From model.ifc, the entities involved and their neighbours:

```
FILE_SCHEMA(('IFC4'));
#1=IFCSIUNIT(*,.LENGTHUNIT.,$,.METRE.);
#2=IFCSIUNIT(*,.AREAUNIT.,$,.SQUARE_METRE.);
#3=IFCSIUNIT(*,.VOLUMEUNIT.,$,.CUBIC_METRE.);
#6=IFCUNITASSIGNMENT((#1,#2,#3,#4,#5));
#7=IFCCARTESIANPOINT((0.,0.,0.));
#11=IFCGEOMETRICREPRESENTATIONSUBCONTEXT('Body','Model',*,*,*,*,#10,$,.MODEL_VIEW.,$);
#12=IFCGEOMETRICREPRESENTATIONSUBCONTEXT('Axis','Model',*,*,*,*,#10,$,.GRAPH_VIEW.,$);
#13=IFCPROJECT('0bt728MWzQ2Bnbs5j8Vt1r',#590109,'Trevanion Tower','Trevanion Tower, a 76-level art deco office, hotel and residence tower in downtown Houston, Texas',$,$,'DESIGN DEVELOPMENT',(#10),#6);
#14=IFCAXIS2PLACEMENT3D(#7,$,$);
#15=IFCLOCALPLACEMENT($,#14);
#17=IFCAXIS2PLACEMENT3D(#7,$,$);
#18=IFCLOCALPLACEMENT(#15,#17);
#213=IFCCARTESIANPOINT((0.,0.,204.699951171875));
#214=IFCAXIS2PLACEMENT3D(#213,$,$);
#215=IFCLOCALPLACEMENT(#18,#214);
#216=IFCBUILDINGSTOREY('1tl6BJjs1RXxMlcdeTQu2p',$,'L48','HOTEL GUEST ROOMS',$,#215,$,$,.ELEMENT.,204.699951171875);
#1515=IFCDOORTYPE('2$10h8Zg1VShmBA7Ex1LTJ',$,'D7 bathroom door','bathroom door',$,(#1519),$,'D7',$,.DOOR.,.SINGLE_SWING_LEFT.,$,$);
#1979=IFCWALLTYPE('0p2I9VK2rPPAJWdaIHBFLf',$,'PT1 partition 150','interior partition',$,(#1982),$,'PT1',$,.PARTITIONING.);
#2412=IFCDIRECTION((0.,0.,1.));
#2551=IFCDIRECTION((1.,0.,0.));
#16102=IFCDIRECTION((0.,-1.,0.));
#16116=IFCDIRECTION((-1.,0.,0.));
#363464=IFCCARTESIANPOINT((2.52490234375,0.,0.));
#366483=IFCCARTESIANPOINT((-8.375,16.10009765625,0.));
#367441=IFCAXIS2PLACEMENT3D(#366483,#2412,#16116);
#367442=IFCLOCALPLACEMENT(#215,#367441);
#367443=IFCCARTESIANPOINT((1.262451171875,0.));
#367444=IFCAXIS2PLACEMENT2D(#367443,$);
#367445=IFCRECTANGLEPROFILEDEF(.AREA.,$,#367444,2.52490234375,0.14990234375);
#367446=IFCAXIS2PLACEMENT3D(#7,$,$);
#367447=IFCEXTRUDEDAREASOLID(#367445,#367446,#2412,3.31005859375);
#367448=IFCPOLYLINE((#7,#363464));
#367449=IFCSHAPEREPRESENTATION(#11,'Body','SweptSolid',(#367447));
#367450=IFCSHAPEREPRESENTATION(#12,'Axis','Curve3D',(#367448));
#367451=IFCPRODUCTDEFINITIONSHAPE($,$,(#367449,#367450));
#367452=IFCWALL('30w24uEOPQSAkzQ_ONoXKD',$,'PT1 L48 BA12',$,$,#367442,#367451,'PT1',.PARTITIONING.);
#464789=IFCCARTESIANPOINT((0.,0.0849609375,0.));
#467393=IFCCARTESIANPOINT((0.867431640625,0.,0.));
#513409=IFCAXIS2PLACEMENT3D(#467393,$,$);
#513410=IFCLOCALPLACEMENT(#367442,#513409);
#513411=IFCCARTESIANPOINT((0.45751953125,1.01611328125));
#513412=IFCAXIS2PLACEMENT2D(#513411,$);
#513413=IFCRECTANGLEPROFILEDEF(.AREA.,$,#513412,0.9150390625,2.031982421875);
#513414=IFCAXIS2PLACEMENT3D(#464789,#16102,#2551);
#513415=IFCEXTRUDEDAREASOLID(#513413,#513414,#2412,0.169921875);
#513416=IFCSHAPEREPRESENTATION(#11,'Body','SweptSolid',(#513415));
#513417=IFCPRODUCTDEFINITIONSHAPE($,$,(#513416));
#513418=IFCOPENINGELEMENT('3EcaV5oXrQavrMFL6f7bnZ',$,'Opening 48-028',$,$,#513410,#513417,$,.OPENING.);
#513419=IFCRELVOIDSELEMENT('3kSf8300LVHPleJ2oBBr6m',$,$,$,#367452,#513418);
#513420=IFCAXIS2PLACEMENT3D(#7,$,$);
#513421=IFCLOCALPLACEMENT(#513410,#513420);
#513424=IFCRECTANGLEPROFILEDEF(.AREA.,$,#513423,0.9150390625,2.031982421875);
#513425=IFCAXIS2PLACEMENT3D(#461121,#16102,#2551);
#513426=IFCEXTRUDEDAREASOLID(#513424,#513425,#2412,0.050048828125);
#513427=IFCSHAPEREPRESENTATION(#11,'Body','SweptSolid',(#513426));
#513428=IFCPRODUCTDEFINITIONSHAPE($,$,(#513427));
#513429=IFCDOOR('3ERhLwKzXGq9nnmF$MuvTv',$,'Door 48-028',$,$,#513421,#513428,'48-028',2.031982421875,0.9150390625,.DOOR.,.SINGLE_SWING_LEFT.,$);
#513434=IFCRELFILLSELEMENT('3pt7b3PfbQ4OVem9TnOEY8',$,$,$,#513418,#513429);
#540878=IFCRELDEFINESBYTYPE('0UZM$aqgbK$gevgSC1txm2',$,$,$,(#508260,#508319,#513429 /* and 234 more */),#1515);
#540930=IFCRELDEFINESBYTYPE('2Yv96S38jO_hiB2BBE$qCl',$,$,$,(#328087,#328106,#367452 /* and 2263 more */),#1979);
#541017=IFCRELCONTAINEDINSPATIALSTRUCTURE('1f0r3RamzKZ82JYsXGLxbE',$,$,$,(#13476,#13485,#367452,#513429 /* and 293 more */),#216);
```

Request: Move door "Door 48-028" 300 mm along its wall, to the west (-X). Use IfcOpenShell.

```python
import ifcopenshell
import ifcopenshell.api.geometry
import ifcopenshell.util.placement
import ifcopenshell.util.unit

model = ifcopenshell.open("model.ifc")
unit_scale = ifcopenshell.util.unit.calculate_unit_scale(model)

door = model.by_id(513429)
opening = door.FillsVoids[0].RelatingOpeningElement
wall = opening.VoidsElements[0].RelatingBuildingElement

wall_matrix = ifcopenshell.util.placement.get_local_placement(wall.ObjectPlacement)
shift = wall_matrix[:3, 0] * 0.3 / unit_scale
before = ifcopenshell.util.placement.get_local_placement(door.ObjectPlacement)[:3, 3].copy()

# The door is placed relative to its opening, so it follows when the opening moves.
matrix = ifcopenshell.util.placement.get_local_placement(opening.ObjectPlacement)
matrix[:3, 3] += shift
ifcopenshell.api.geometry.edit_object_placement(
    model, product=opening, matrix=matrix, is_si=False, should_transform_children=True
)

after = ifcopenshell.util.placement.get_local_placement(door.ObjectPlacement)[:3, 3]
print("door moved by", (after - before).round(3) + 0.0)

model.write("model_v2.ifc")
```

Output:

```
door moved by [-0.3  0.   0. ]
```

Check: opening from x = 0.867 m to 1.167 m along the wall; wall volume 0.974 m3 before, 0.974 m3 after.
